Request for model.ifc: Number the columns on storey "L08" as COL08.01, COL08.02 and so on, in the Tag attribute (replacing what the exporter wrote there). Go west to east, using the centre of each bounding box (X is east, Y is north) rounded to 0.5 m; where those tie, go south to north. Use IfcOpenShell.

First a look at what the model holds.

```python
import ifcopenshell
import ifcopenshell.util.element
import ifcopenshell.util.placement

model = ifcopenshell.open("model.ifc")
print(model.schema)
storey = next(s for s in model.by_type("IfcBuildingStorey") if s.Name == "L08")
columns = [e for e in ifcopenshell.util.element.get_decomposition(storey) if e.is_a("IfcColumn")]
for e in sorted(columns, key=lambda e: e.id()):
    origin = ifcopenshell.util.placement.get_local_placement(e.ObjectPlacement)[:3, 3]
    print(e.id(), e.Tag, e.Name, origin.round(2) + 0.0, sep=" | ")
```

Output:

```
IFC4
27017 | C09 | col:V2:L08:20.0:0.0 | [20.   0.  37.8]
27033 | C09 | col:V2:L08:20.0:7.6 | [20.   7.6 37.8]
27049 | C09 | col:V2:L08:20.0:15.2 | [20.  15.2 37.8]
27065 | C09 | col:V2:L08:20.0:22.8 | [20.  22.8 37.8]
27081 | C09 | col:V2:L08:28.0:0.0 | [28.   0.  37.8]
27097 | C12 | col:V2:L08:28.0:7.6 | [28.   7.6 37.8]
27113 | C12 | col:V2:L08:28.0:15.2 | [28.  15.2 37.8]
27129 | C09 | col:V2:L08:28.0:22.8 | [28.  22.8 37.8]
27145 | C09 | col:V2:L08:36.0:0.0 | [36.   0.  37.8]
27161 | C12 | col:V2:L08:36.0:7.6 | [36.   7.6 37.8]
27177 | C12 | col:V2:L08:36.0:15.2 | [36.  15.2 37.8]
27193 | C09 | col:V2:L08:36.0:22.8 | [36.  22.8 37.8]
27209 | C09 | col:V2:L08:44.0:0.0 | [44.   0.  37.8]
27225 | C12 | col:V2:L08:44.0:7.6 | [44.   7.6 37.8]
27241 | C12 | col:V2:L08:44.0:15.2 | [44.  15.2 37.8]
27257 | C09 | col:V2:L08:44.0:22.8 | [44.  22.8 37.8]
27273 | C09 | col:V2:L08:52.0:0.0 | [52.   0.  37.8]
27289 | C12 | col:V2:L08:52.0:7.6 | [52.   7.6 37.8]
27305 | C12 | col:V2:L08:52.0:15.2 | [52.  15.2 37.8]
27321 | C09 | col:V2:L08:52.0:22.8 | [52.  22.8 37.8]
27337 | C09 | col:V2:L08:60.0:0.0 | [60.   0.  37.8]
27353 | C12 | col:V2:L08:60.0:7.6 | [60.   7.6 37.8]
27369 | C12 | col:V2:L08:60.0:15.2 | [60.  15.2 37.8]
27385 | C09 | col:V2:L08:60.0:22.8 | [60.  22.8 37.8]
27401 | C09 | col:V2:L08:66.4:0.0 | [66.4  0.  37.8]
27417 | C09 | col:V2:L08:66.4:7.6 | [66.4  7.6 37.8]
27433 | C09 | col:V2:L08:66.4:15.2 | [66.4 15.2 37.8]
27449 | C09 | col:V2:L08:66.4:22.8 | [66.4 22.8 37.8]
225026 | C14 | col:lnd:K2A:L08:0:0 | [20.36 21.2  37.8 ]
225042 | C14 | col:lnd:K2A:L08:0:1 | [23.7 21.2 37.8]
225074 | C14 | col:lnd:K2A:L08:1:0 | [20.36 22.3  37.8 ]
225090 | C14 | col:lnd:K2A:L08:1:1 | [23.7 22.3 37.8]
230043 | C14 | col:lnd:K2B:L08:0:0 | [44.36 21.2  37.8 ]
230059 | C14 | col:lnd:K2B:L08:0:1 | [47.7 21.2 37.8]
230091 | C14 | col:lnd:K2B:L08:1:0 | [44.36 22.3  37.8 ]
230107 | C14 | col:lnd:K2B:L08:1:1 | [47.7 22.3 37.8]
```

```python
import ifcopenshell
import ifcopenshell.geom
import ifcopenshell.util.element
import ifcopenshell.util.shape

model = ifcopenshell.open("model.ifc")
settings = ifcopenshell.geom.settings()
settings.set("use-world-coords", True)


def centre(element):
    shape = ifcopenshell.geom.create_shape(settings, element)
    return ifcopenshell.util.shape.get_bbox_centroid(shape.geometry)


storey = next(s for s in model.by_type("IfcBuildingStorey") if s.Name == "L08")
columns = [e for e in ifcopenshell.util.element.get_decomposition(storey) if e.is_a("IfcColumn")]

# Insertion points can sit at a corner or the storey origin, so sort by the geometry (in metres).
centres = {e: centre(e) for e in columns}
columns.sort(key=lambda e: (round(centres[e][0] / 0.5), centres[e][1]))

for i, e in enumerate(columns, start=1):
    number = f"COL08.{i:02d}"
    e.Tag = number
    print(e.id(), number)

model.write("model_rev.ifc")
```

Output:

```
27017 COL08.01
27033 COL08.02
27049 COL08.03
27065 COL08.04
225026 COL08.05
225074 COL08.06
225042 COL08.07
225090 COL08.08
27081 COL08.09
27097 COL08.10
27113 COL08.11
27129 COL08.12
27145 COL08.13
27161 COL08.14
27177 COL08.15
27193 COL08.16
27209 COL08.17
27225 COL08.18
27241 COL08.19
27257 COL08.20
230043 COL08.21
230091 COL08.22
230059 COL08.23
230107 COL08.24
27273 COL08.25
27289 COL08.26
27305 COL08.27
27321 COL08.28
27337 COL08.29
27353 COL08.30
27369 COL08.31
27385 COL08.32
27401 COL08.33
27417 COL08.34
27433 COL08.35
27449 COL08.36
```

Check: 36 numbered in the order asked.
